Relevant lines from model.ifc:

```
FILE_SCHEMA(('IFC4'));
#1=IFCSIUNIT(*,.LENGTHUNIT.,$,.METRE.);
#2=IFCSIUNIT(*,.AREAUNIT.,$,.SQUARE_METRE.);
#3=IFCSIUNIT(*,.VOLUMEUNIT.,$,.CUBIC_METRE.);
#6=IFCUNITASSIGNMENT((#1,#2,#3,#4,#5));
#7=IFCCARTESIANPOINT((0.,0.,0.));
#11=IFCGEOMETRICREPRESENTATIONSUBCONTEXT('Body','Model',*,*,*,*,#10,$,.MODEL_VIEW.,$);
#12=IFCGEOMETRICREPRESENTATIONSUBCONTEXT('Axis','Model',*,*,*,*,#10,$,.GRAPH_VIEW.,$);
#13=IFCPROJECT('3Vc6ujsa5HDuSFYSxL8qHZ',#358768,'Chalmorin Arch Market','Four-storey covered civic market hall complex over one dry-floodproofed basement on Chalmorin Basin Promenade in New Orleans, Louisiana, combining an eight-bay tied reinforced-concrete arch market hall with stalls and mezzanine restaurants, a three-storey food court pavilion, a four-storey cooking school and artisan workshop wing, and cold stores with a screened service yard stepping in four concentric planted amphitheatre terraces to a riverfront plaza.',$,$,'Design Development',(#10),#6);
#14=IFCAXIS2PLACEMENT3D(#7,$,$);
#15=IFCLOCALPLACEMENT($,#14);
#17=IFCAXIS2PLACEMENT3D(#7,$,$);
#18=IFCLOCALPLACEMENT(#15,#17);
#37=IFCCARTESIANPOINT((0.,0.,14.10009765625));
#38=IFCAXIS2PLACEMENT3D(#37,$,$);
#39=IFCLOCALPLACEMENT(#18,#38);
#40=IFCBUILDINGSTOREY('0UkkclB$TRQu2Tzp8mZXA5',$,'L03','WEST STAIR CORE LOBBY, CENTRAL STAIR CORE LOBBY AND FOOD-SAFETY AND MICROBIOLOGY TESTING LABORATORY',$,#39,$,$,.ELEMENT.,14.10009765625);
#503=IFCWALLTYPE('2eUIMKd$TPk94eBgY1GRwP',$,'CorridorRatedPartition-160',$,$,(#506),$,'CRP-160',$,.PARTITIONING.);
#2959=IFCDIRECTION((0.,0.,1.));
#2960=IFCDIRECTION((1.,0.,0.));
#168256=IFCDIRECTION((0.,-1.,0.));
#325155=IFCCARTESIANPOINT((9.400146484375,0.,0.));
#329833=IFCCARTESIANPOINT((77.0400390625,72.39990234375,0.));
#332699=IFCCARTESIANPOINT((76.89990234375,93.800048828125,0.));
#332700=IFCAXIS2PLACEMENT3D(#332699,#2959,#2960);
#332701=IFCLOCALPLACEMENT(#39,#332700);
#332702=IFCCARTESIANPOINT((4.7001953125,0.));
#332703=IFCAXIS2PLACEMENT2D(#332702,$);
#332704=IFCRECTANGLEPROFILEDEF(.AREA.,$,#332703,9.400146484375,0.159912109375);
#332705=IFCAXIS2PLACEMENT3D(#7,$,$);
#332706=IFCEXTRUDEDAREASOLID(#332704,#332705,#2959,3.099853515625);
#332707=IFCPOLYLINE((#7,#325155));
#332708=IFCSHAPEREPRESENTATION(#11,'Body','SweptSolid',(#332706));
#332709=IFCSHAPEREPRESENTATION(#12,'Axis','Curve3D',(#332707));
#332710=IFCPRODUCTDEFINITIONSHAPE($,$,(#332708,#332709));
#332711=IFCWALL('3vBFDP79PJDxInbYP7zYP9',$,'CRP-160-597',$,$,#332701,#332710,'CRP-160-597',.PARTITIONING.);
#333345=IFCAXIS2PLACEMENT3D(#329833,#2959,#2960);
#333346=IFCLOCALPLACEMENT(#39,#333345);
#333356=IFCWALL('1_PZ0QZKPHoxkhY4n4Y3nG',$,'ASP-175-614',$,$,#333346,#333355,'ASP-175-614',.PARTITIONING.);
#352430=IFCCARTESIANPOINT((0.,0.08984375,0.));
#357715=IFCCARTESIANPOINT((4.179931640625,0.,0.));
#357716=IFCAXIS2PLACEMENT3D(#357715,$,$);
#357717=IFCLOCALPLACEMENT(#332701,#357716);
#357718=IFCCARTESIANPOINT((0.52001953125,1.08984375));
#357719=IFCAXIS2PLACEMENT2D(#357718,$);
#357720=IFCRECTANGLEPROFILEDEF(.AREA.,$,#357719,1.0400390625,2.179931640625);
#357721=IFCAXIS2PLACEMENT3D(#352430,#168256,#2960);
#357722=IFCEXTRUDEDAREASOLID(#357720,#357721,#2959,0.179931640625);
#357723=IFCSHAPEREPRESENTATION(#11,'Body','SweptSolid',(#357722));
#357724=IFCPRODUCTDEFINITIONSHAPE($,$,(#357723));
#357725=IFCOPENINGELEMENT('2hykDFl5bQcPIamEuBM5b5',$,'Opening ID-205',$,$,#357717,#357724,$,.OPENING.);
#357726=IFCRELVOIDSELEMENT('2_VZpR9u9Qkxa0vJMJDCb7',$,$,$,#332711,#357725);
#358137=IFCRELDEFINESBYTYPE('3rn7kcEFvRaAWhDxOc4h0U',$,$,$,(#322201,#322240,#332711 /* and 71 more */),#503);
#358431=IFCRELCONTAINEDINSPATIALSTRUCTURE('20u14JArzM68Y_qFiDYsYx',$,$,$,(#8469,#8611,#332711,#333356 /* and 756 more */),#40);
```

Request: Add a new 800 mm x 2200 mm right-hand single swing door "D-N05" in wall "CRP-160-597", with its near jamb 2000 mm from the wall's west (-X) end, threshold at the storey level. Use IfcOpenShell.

```python
import numpy as np
import ifcopenshell
import ifcopenshell.api.feature
import ifcopenshell.api.geometry
import ifcopenshell.api.root
import ifcopenshell.api.spatial
import ifcopenshell.geom
import ifcopenshell.util.element
import ifcopenshell.util.placement
import ifcopenshell.util.representation
import ifcopenshell.util.shape
import ifcopenshell.util.unit

model = ifcopenshell.open("model.ifc")
unit_scale = ifcopenshell.util.unit.calculate_unit_scale(model)
settings = ifcopenshell.geom.settings()


def volume(element):
    """Net volume in cubic metres, openings subtracted."""
    shape = ifcopenshell.geom.create_shape(settings, element)
    return ifcopenshell.util.shape.get_volume(shape.geometry)


wall = model.by_guid("3vBFDP79PJDxInbYP7zYP9")
storey = ifcopenshell.util.element.get_container(wall, ifc_class="IfcBuildingStorey")
context = ifcopenshell.util.representation.get_context(model, "Model", "Body", "MODEL_VIEW")
before = volume(wall)

width, height, from_end, sill = 0.8, 2.2, 2, 0.0  # metres

# The wall runs along its own X axis, and the end named is its -X end.
wall_shape = ifcopenshell.geom.create_shape(settings, wall)
x, y, z = ifcopenshell.util.shape.get_vertices(wall_shape.geometry).T
start = x.min() + from_end
face, thickness = float(y.min()), float(y.max() - y.min())
wall_matrix = ifcopenshell.util.placement.get_local_placement(wall.ObjectPlacement)
level = ifcopenshell.util.placement.get_local_placement(storey.ObjectPlacement)[2, 3]


def in_wall(x, y):
    """Placement at x, y metres in the wall's axes, at sill height."""
    matrix = wall_matrix.copy()
    matrix[:, 3] = wall_matrix @ np.array([x / unit_scale, y / unit_scale, 0.0, 1.0])
    matrix[2, 3] = level + sill / unit_scale
    return matrix


# Opening: a box that overshoots both wall faces by 50 mm.
opening = ifcopenshell.api.root.create_entity(model, ifc_class="IfcOpeningElement", predefined_type="OPENING")
box = ifcopenshell.api.geometry.add_wall_representation(
    model, context=context, length=width, height=height, thickness=thickness + 0.1
)
ifcopenshell.api.geometry.assign_representation(model, product=opening, representation=box)
ifcopenshell.api.geometry.edit_object_placement(model, product=opening, matrix=in_wall(start, face - 0.05), is_si=False)
ifcopenshell.api.feature.add_feature(model, feature=opening, element=wall)

door = ifcopenshell.api.root.create_entity(model, ifc_class="IfcDoor", name="D-N05", predefined_type="DOOR")
door.OverallWidth, door.OverallHeight = width / unit_scale, height / unit_scale
door.OperationType = "SINGLE_SWING_RIGHT"
body = ifcopenshell.api.geometry.add_door_representation(
    model,
    context=context,
    overall_width=door.OverallWidth,
    overall_height=door.OverallHeight,
    operation_type="SINGLE_SWING_RIGHT",
    lining_properties={"LiningDepth": thickness / unit_scale, "ThresholdDepth": thickness / unit_scale},
)
ifcopenshell.api.geometry.assign_representation(model, product=door, representation=body)
ifcopenshell.api.spatial.assign_container(model, products=[door], relating_structure=storey)
ifcopenshell.api.feature.add_filling(model, opening=opening, element=door)

# The lining spans the wall, so the door starts at the wall face.
ifcopenshell.api.geometry.edit_object_placement(model, product=door, matrix=in_wall(start, face), is_si=False)

after = volume(wall)

print(f"wall volume {before:.3f} -> {after:.3f} m3")

model.write("model_v2.ifc")
```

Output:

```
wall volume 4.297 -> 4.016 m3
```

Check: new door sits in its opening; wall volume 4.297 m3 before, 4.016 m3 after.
